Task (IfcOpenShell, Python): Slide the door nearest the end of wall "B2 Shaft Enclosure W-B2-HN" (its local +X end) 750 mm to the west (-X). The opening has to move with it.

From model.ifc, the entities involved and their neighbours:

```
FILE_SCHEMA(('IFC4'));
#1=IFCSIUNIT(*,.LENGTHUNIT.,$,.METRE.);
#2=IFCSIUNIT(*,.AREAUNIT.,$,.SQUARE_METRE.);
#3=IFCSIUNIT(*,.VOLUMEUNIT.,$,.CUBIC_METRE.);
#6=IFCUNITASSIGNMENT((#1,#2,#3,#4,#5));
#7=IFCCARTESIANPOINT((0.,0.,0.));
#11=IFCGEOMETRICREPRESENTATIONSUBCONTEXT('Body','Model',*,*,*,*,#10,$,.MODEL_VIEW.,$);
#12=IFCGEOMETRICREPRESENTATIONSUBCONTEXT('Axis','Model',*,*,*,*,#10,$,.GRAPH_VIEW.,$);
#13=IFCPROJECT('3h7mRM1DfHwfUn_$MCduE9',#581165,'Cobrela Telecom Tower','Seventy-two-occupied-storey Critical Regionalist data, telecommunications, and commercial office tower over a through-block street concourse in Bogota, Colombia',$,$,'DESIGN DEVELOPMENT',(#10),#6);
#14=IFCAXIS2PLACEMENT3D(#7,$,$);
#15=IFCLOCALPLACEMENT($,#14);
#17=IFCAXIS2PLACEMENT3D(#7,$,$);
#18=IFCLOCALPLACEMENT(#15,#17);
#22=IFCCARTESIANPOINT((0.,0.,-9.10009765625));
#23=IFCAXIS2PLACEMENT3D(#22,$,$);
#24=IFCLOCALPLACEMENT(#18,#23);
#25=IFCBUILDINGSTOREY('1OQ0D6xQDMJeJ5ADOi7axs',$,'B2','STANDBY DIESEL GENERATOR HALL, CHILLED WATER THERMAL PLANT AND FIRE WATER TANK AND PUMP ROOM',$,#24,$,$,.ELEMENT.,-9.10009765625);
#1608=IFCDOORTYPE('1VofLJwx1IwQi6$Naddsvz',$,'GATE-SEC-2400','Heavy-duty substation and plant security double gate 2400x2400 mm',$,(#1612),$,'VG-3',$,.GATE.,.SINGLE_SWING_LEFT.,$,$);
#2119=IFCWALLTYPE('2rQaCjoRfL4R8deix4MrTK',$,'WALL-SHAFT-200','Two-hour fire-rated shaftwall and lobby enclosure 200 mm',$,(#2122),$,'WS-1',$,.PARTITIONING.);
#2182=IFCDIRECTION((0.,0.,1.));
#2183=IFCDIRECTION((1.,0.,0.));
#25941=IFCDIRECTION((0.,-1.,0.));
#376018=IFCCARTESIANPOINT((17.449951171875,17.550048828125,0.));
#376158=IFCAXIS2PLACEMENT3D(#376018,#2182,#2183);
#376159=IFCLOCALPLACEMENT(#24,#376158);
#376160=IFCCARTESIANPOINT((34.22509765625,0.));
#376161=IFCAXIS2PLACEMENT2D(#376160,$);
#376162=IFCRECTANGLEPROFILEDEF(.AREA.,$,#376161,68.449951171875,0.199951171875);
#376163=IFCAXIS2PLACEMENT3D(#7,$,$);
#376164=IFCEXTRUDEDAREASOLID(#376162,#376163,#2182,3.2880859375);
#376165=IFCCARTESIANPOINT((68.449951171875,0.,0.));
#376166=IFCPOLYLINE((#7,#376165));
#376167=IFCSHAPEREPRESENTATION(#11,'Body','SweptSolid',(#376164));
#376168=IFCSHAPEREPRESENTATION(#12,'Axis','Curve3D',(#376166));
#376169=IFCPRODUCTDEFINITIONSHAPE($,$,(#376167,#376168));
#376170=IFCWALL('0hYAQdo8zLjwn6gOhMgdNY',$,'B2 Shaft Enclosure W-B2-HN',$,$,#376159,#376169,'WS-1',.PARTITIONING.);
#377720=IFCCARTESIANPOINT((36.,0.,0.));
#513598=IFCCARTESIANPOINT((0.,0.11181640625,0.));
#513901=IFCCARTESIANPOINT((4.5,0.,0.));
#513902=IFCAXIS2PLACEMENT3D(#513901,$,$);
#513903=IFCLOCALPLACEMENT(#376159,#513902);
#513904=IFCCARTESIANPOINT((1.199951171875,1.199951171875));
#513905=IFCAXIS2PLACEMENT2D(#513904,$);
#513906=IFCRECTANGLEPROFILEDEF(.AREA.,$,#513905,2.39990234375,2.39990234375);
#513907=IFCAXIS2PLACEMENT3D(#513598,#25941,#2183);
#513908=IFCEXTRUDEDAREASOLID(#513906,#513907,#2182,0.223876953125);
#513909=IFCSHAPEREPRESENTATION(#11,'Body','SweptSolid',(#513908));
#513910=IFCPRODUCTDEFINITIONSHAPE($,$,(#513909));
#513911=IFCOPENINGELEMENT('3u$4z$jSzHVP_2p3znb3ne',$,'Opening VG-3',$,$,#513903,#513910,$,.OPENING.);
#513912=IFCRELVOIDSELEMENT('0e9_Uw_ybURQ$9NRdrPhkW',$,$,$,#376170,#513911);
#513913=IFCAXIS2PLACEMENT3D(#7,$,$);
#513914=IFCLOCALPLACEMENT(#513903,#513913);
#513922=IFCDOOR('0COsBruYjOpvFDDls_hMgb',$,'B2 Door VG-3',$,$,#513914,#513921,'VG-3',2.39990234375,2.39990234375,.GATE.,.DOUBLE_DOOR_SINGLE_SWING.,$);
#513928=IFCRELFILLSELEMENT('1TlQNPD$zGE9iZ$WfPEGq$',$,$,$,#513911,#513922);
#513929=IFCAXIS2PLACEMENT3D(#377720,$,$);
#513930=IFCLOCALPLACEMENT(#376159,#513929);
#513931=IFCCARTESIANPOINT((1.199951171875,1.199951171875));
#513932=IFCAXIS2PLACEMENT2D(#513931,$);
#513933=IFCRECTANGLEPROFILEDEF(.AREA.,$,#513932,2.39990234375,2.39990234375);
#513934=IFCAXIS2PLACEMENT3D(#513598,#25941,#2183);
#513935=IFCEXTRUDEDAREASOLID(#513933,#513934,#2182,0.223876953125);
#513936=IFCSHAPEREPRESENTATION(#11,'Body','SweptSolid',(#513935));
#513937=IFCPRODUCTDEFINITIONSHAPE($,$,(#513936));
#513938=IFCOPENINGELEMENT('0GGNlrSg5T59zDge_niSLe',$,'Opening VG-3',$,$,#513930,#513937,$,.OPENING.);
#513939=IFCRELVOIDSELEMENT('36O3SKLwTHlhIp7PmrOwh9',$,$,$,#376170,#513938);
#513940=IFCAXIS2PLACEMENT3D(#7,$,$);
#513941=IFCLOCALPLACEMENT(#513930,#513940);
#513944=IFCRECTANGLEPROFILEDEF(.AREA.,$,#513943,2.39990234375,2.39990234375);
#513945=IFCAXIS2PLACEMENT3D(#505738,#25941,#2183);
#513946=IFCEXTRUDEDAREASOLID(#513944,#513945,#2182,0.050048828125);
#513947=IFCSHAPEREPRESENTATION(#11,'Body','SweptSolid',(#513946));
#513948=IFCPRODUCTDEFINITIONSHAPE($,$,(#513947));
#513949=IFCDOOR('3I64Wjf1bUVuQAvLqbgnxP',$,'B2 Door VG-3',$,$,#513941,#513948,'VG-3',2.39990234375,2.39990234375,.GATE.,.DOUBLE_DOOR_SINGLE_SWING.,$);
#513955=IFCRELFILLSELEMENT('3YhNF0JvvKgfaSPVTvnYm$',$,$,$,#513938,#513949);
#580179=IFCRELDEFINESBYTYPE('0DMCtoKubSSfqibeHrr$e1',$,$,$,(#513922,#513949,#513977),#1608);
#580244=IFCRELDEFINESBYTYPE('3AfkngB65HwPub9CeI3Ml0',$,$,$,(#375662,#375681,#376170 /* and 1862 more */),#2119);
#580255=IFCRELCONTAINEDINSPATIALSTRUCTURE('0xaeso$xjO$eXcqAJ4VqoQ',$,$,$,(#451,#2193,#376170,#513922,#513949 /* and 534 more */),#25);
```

```python
import ifcopenshell
import ifcopenshell.api.geometry
import ifcopenshell.util.placement
import ifcopenshell.util.unit

model = ifcopenshell.open("model.ifc")
unit_scale = ifcopenshell.util.unit.calculate_unit_scale(model)

door = model.by_guid("3I64Wjf1bUVuQAvLqbgnxP")
opening = door.FillsVoids[0].RelatingOpeningElement
wall = opening.VoidsElements[0].RelatingBuildingElement

wall_matrix = ifcopenshell.util.placement.get_local_placement(wall.ObjectPlacement)
shift = wall_matrix[:3, 0] * -0.75 / unit_scale
before = ifcopenshell.util.placement.get_local_placement(door.ObjectPlacement)[:3, 3].copy()

# The door is placed relative to its opening, so it follows when the opening moves.
matrix = ifcopenshell.util.placement.get_local_placement(opening.ObjectPlacement)
matrix[:3, 3] += shift
ifcopenshell.api.geometry.edit_object_placement(
    model, product=opening, matrix=matrix, is_si=False, should_transform_children=True
)

after = ifcopenshell.util.placement.get_local_placement(door.ObjectPlacement)[:3, 3]
print("door moved by", (after - before).round(3) + 0.0)

model.write("model-out.ifc")
```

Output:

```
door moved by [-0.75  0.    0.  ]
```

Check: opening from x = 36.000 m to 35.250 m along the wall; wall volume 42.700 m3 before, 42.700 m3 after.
